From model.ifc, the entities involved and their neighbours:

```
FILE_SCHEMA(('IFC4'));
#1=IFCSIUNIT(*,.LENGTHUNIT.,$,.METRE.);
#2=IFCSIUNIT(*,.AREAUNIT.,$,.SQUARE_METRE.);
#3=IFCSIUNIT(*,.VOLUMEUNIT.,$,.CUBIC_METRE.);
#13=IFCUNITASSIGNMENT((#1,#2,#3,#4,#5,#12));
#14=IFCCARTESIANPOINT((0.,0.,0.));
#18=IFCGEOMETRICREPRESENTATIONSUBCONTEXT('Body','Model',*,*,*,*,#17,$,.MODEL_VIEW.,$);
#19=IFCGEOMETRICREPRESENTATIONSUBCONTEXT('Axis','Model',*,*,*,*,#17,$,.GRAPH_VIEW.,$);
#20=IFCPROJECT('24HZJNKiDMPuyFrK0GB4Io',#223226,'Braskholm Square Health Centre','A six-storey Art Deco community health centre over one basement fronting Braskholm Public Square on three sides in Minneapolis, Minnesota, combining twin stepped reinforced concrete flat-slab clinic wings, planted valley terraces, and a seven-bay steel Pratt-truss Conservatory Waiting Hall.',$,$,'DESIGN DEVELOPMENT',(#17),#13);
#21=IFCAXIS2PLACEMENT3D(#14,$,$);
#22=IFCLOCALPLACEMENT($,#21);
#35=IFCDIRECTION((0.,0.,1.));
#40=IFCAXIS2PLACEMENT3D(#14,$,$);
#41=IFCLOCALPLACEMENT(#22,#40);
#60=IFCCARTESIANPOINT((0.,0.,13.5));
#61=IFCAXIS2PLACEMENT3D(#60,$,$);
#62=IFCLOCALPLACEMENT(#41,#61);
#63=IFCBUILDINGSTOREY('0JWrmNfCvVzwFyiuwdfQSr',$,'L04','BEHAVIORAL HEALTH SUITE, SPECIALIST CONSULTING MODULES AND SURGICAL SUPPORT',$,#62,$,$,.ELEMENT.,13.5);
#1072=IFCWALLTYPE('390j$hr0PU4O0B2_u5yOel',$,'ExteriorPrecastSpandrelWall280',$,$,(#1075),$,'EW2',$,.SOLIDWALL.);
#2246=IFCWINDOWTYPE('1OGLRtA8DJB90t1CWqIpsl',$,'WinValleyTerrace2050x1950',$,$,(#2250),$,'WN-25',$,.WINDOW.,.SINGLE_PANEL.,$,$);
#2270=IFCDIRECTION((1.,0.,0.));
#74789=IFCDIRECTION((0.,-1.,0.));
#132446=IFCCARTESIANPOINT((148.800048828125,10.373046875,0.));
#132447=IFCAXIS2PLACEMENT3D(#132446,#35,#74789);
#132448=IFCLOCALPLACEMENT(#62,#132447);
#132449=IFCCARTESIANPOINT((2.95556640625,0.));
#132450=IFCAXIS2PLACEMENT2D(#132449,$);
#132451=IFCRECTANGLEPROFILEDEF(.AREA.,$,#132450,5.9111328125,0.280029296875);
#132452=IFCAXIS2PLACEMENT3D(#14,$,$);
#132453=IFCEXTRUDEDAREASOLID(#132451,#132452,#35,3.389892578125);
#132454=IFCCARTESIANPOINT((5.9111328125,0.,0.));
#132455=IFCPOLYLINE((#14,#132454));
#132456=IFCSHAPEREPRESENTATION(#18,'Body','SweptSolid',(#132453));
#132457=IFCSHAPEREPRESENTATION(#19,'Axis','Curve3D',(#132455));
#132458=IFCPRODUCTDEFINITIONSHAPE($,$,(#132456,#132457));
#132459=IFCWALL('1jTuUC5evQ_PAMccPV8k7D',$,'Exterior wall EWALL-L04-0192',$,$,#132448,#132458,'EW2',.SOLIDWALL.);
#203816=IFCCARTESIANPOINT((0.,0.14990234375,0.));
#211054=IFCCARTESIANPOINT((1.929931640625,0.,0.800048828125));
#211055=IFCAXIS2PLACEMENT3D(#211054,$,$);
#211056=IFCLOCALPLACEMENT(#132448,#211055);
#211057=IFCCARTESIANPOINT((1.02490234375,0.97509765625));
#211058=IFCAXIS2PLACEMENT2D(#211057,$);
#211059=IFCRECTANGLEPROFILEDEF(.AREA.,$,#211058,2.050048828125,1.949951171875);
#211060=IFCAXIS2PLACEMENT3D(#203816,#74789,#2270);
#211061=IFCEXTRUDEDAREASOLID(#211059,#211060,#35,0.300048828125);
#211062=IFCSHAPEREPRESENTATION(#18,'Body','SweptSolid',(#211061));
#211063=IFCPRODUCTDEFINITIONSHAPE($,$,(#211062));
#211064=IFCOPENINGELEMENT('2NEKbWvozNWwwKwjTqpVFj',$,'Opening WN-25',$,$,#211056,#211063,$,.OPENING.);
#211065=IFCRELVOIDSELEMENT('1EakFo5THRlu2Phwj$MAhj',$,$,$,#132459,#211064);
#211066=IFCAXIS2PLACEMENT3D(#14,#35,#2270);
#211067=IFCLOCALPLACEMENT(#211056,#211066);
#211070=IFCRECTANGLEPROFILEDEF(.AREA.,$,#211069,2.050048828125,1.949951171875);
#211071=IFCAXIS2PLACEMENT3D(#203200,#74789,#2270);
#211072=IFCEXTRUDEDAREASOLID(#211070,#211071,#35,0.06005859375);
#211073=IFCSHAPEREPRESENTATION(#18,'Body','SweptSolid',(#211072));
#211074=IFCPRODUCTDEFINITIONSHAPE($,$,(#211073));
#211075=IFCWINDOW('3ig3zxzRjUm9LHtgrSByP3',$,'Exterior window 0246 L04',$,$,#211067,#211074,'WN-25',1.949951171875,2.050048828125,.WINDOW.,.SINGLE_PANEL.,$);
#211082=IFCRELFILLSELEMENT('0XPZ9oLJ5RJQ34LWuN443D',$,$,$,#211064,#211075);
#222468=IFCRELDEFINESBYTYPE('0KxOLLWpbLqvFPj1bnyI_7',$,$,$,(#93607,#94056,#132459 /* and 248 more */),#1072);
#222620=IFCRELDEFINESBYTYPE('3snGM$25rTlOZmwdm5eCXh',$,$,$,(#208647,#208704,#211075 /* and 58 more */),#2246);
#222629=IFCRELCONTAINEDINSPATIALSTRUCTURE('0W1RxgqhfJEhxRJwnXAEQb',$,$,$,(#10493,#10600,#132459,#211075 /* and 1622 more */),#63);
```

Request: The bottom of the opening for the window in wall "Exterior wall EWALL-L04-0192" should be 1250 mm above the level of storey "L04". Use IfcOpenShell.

```python
import numpy as np
import ifcopenshell
import ifcopenshell.api.geometry
import ifcopenshell.geom
import ifcopenshell.util.element
import ifcopenshell.util.placement
import ifcopenshell.util.shape
import ifcopenshell.util.unit

model = ifcopenshell.open("model.ifc")
unit_scale = ifcopenshell.util.unit.calculate_unit_scale(model)

window = model.by_guid("3ig3zxzRjUm9LHtgrSByP3")
opening = window.FillsVoids[0].RelatingOpeningElement
storey = ifcopenshell.util.element.get_container(window, ifc_class="IfcBuildingStorey")
level = ifcopenshell.util.placement.get_local_placement(storey.ObjectPlacement)[2, 3]

# The opening's origin need not be at the sill, so measure its lowest point.
shape = ifcopenshell.geom.create_shape(ifcopenshell.geom.settings(), opening)
bottom = ifcopenshell.util.shape.get_shape_bottom_elevation(shape, shape.geometry) / unit_scale
dz = level + 1.25 / unit_scale - bottom

shift = np.array([0.0, 0.0, dz])
# The window is placed relative to its opening, so it follows when the opening moves.
matrix = ifcopenshell.util.placement.get_local_placement(opening.ObjectPlacement)
matrix[:3, 3] += shift
ifcopenshell.api.geometry.edit_object_placement(
    model, product=opening, matrix=matrix, is_si=False, should_transform_children=True
)

print(f"moved by {dz * unit_scale:+.3f} m")

model.write("model_v2.ifc")
```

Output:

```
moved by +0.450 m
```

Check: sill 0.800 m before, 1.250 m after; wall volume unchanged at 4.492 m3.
